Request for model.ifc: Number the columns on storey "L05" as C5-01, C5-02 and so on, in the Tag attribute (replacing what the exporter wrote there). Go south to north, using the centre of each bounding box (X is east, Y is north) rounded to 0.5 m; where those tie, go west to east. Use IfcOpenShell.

First a look at what the model holds.

```python
import ifcopenshell
import ifcopenshell.util.element
import ifcopenshell.util.placement

model = ifcopenshell.open("model.ifc")
print(model.schema)
storey = next(s for s in model.by_type("IfcBuildingStorey") if s.Name == "L05")
columns = [e for e in ifcopenshell.util.element.get_decomposition(storey) if e.is_a("IfcColumn")]
for e in sorted(columns, key=lambda e: e.id()):
    origin = ifcopenshell.util.placement.get_local_placement(e.ObjectPlacement)[:3, 3]
    print(e.id(), e.Tag, e.Name, origin.round(2) + 0.0, sep=" | ")
```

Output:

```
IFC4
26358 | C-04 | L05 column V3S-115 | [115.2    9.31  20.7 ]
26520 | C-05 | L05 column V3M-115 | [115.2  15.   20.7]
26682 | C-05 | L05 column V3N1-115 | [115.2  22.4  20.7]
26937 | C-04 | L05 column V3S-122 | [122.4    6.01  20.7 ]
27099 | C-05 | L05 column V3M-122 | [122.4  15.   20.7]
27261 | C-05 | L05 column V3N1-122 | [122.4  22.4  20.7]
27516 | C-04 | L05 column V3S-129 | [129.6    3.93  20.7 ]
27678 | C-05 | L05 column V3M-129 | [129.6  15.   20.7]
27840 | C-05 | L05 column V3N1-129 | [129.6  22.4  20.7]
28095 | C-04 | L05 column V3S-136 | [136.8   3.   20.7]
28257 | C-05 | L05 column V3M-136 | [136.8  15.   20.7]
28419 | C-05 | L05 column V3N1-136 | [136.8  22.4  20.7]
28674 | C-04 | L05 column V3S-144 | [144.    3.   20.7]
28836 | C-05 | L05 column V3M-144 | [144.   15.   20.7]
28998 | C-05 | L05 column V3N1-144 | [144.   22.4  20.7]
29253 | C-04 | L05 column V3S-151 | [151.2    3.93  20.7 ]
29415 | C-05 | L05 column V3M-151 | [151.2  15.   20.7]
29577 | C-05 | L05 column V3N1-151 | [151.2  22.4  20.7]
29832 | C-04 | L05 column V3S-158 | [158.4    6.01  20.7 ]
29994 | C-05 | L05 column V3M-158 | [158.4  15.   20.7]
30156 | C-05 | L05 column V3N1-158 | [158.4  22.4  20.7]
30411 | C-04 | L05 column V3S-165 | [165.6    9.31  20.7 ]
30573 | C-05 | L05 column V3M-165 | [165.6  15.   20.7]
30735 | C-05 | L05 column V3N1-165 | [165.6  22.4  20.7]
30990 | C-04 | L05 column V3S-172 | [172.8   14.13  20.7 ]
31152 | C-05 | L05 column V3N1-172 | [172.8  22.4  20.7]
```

```python
import ifcopenshell
import ifcopenshell.geom
import ifcopenshell.util.element
import ifcopenshell.util.shape

model = ifcopenshell.open("model.ifc")
settings = ifcopenshell.geom.settings()
settings.set("use-world-coords", True)


def centre(element):
    shape = ifcopenshell.geom.create_shape(settings, element)
    return ifcopenshell.util.shape.get_bbox_centroid(shape.geometry)


storey = next(s for s in model.by_type("IfcBuildingStorey") if s.Name == "L05")
columns = [e for e in ifcopenshell.util.element.get_decomposition(storey) if e.is_a("IfcColumn")]

# Insertion points can sit at a corner or the storey origin, so sort by the geometry (in metres).
centres = {e: centre(e) for e in columns}
columns.sort(key=lambda e: (round(centres[e][1] / 0.5), centres[e][0]))

for i, e in enumerate(columns, start=1):
    number = f"C5-{i:02d}"
    e.Tag = number
    print(e.id(), number)

model.write("model-out.ifc")
```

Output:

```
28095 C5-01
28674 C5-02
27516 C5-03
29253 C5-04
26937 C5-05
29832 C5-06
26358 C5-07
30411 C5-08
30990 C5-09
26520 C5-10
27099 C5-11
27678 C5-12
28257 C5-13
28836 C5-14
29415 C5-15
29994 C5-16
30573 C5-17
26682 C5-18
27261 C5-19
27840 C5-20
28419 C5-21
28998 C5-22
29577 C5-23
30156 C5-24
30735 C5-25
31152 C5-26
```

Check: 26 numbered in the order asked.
